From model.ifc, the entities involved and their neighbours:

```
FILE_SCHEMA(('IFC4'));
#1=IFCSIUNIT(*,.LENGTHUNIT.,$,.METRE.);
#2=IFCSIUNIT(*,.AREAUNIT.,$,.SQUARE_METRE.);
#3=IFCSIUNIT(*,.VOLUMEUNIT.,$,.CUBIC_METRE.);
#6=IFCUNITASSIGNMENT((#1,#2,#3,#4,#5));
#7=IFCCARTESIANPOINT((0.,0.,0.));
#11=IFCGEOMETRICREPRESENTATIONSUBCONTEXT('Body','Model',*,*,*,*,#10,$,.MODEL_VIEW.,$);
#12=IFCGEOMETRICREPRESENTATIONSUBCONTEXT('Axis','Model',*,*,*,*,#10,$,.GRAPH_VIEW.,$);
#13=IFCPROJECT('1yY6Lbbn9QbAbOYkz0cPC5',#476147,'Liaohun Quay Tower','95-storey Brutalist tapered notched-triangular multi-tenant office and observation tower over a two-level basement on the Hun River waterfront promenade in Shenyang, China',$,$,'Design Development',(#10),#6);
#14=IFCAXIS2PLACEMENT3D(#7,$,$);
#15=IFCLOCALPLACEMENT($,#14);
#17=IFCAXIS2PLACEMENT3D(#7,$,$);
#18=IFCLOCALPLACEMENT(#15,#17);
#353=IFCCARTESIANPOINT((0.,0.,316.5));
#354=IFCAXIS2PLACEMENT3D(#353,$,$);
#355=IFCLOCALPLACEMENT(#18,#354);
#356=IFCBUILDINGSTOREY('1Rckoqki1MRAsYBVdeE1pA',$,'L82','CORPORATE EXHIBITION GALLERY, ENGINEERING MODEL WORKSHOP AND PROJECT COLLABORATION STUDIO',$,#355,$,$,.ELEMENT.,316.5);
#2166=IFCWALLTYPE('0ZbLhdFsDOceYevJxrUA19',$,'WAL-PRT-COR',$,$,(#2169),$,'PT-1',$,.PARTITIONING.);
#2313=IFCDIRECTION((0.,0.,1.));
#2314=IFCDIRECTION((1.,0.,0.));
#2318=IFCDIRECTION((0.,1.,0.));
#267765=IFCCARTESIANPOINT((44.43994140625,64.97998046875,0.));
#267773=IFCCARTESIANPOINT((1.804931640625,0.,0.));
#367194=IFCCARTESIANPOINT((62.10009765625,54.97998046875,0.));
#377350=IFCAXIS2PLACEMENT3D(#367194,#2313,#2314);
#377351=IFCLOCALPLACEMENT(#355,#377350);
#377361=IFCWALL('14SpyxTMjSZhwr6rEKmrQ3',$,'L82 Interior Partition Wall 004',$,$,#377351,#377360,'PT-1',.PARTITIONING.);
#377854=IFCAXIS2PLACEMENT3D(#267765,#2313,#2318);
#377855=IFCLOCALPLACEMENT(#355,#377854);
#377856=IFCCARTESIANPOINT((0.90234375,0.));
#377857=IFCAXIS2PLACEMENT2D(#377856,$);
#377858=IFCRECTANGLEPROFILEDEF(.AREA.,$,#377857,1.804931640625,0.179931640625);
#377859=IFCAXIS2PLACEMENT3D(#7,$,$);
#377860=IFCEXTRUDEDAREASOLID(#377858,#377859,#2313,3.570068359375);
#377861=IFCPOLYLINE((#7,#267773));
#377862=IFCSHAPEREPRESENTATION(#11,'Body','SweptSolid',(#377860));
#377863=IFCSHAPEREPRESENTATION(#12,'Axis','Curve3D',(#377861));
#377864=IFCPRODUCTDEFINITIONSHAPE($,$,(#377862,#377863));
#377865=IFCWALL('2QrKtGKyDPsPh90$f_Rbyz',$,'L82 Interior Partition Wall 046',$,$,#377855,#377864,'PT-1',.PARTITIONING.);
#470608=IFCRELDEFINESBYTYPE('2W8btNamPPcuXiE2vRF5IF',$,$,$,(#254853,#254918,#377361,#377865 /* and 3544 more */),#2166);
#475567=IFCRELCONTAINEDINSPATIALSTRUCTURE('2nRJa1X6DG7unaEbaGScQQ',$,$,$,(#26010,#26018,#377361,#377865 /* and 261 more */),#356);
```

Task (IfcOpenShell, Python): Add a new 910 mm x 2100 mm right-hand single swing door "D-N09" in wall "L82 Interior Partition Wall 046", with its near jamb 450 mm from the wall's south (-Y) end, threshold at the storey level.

```python
import numpy as np
import ifcopenshell
import ifcopenshell.api.feature
import ifcopenshell.api.geometry
import ifcopenshell.api.root
import ifcopenshell.api.spatial
import ifcopenshell.geom
import ifcopenshell.util.element
import ifcopenshell.util.placement
import ifcopenshell.util.representation
import ifcopenshell.util.shape
import ifcopenshell.util.unit

model = ifcopenshell.open("model.ifc")
unit_scale = ifcopenshell.util.unit.calculate_unit_scale(model)
settings = ifcopenshell.geom.settings()


def volume(element):
    """Net volume in cubic metres, openings subtracted."""
    shape = ifcopenshell.geom.create_shape(settings, element)
    return ifcopenshell.util.shape.get_volume(shape.geometry)


wall = model.by_guid("2QrKtGKyDPsPh90$f_Rbyz")
storey = ifcopenshell.util.element.get_container(wall, ifc_class="IfcBuildingStorey")
context = ifcopenshell.util.representation.get_context(model, "Model", "Body", "MODEL_VIEW")
before = volume(wall)

width, height, from_end, sill = 0.91, 2.1, 0.45, 0.0  # metres

# The wall runs along its own X axis, and the end named is its -X end.
wall_shape = ifcopenshell.geom.create_shape(settings, wall)
x, y, z = ifcopenshell.util.shape.get_vertices(wall_shape.geometry).T
start = x.min() + from_end
face, thickness = float(y.min()), float(y.max() - y.min())
wall_matrix = ifcopenshell.util.placement.get_local_placement(wall.ObjectPlacement)
level = ifcopenshell.util.placement.get_local_placement(storey.ObjectPlacement)[2, 3]


def in_wall(x, y):
    """Placement at x, y metres in the wall's axes, at sill height."""
    matrix = wall_matrix.copy()
    matrix[:, 3] = wall_matrix @ np.array([x / unit_scale, y / unit_scale, 0.0, 1.0])
    matrix[2, 3] = level + sill / unit_scale
    return matrix


# Opening: a box that overshoots both wall faces by 50 mm.
opening = ifcopenshell.api.root.create_entity(model, ifc_class="IfcOpeningElement", predefined_type="OPENING")
box = ifcopenshell.api.geometry.add_wall_representation(
    model, context=context, length=width, height=height, thickness=thickness + 0.1
)
ifcopenshell.api.geometry.assign_representation(model, product=opening, representation=box)
ifcopenshell.api.geometry.edit_object_placement(model, product=opening, matrix=in_wall(start, face - 0.05), is_si=False)
ifcopenshell.api.feature.add_feature(model, feature=opening, element=wall)

door = ifcopenshell.api.root.create_entity(model, ifc_class="IfcDoor", name="D-N09", predefined_type="DOOR")
door.OverallWidth, door.OverallHeight = width / unit_scale, height / unit_scale
door.OperationType = "SINGLE_SWING_RIGHT"
body = ifcopenshell.api.geometry.add_door_representation(
    model,
    context=context,
    overall_width=door.OverallWidth,
    overall_height=door.OverallHeight,
    operation_type="SINGLE_SWING_RIGHT",
    lining_properties={"LiningDepth": thickness / unit_scale, "ThresholdDepth": thickness / unit_scale},
)
ifcopenshell.api.geometry.assign_representation(model, product=door, representation=body)
ifcopenshell.api.spatial.assign_container(model, products=[door], relating_structure=storey)
ifcopenshell.api.feature.add_filling(model, opening=opening, element=door)

# The lining spans the wall, so the door starts at the wall face.
ifcopenshell.api.geometry.edit_object_placement(model, product=door, matrix=in_wall(start, face), is_si=False)

after = volume(wall)

print(f"wall volume {before:.3f} -> {after:.3f} m3")

model.write("model_edited.ifc")
```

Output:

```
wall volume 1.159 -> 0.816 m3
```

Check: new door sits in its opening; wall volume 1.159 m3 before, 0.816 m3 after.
